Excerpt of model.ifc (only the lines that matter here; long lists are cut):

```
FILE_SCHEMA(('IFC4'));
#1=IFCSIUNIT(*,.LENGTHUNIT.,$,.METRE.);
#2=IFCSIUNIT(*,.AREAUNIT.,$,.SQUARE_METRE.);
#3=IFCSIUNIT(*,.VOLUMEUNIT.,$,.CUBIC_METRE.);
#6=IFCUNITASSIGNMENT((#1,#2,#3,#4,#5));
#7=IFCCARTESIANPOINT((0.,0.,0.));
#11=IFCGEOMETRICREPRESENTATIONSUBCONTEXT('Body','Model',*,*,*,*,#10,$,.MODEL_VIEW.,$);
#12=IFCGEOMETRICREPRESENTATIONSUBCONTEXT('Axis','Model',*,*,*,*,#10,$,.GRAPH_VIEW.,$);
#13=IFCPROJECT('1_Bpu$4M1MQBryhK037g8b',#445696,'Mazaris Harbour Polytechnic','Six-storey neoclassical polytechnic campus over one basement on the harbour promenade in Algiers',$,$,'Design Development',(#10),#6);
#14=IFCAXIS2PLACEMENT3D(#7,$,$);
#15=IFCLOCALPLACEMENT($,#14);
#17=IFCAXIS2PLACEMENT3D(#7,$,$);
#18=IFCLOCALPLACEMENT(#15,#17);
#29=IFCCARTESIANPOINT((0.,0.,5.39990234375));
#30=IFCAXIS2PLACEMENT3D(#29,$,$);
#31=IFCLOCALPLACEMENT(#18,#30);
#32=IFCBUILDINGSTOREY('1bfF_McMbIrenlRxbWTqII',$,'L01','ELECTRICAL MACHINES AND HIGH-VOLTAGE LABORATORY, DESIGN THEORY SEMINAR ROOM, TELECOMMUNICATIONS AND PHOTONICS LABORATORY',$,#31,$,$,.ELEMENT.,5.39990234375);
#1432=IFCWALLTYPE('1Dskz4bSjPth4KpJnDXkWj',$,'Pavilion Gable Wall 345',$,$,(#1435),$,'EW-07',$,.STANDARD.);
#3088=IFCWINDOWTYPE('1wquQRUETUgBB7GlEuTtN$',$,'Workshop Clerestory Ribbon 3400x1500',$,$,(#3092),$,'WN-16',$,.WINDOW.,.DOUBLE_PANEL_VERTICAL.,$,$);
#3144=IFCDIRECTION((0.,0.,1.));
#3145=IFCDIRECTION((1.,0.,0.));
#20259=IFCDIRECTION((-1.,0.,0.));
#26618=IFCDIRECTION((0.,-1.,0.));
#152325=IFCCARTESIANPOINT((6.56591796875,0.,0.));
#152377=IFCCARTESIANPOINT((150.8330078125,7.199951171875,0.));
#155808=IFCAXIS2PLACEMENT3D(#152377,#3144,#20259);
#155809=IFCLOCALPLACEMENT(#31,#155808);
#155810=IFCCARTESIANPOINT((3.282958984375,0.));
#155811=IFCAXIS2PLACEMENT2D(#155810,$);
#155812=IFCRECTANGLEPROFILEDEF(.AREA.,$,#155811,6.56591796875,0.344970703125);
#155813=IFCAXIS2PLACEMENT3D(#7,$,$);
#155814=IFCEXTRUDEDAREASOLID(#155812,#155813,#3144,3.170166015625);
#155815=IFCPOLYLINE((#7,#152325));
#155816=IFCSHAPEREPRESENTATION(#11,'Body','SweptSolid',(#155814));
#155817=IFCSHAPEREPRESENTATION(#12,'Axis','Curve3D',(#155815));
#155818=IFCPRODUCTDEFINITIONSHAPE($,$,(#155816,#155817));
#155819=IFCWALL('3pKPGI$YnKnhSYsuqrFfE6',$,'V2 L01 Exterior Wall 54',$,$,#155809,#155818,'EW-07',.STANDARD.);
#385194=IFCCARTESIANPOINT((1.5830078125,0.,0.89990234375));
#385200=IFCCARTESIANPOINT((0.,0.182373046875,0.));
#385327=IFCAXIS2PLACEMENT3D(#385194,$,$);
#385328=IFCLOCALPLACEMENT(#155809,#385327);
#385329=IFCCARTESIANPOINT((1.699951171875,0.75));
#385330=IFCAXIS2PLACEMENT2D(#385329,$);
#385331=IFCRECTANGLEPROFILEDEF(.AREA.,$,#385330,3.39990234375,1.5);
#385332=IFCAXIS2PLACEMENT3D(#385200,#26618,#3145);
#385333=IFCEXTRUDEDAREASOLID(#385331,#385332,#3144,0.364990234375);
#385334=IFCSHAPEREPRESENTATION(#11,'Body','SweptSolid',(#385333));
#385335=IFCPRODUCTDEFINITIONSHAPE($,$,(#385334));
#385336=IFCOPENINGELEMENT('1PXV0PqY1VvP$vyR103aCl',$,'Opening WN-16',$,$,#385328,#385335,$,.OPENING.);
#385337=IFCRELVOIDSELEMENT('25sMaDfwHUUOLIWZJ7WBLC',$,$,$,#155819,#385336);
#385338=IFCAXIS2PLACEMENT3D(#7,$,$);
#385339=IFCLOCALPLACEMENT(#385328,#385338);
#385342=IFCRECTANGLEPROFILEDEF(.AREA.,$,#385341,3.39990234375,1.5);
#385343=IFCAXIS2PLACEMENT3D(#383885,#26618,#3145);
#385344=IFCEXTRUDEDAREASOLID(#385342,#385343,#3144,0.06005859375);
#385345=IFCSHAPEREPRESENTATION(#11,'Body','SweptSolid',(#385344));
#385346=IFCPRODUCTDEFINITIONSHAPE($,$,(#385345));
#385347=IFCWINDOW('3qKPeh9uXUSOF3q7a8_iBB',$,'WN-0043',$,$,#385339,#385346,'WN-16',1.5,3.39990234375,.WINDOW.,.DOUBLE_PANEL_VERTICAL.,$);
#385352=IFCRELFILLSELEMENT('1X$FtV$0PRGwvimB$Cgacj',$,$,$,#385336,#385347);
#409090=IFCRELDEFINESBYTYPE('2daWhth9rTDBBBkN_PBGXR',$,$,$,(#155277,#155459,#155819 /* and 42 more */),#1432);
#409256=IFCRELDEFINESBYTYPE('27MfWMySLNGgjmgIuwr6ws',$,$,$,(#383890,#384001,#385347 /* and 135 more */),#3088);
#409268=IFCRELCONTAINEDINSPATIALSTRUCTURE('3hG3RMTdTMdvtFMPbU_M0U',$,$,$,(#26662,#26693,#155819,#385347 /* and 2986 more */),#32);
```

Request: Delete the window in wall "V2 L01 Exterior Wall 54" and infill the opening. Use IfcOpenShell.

```python
import ifcopenshell
import ifcopenshell.api.feature
import ifcopenshell.api.root
import ifcopenshell.geom
import ifcopenshell.util.shape

model = ifcopenshell.open("model.ifc")
settings = ifcopenshell.geom.settings()


def volume(element):
    """Net volume in cubic metres, openings subtracted."""
    shape = ifcopenshell.geom.create_shape(settings, element)
    return ifcopenshell.util.shape.get_volume(shape.geometry)


window = model.by_guid("3qKPeh9uXUSOF3q7a8_iBB")
opening = window.FillsVoids[0].RelatingOpeningElement
wall = opening.VoidsElements[0].RelatingBuildingElement
before = volume(wall)

ifcopenshell.api.root.remove_product(model, product=window)
ifcopenshell.api.feature.remove_feature(model, feature=opening)

after = volume(wall)

print(f"wall volume {before:.3f} -> {after:.3f} m3")

model.write("model_v2.ifc")
```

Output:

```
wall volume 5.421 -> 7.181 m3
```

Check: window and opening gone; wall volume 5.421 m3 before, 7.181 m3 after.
